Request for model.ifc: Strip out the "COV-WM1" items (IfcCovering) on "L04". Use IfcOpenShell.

First a look at what the model holds.

```python
import ifcopenshell
import ifcopenshell.util.element

model = ifcopenshell.open("model.ifc")
print(model.schema)
storey = next(s for s in model.by_type("IfcBuildingStorey") if s.Name == "L04")
coverings = [e for e in ifcopenshell.util.element.get_decomposition(storey) if e.is_a("IfcCovering")]
seen = {}
for e in coverings:
    element_type = ifcopenshell.util.element.get_type(e)
    name = element_type.Name if element_type not in (None, e) else None
    seen[name] = seen.get(name, 0) + 1
for name, count in sorted(seen.items(), key=str):
    print(count, "x", name)
```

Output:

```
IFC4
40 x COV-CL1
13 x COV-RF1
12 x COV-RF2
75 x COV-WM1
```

```python
import ifcopenshell
import ifcopenshell.api.root
import ifcopenshell.util.element

model = ifcopenshell.open("model.ifc")

storey = next(s for s in model.by_type("IfcBuildingStorey") if s.Name == "L04")
coverings = [e for e in ifcopenshell.util.element.get_decomposition(storey) if e.is_a("IfcCovering")]
targets = [e for e in coverings if (t := ifcopenshell.util.element.get_type(e)) not in (None, e) and t.Name == "COV-WM1"]

for e in targets:
    ifcopenshell.api.root.remove_product(model, product=e)
print(len(targets), "removed")

model.write("model_edited.ifc")
```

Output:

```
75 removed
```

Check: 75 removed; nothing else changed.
